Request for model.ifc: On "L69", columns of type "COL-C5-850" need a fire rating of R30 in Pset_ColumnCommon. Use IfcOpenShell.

First a look at what the model holds.

```python
import ifcopenshell
import ifcopenshell.util.element

model = ifcopenshell.open("model.ifc")
print(model.schema)
storey = next(s for s in model.by_type("IfcBuildingStorey") if s.Name == "L69")
columns = [e for e in ifcopenshell.util.element.get_decomposition(storey) if e.is_a("IfcColumn")]
seen = {}
for e in columns:
    element_type = ifcopenshell.util.element.get_type(e)
    key = (element_type.Name if element_type != e and element_type else None, ifcopenshell.util.element.get_pset(e, "Pset_ColumnCommon", "FireRating"))
    seen[key] = seen.get(key, 0) + 1
for (name, value), count in sorted(seen.items(), key=str):
    print(count, "x", name, "|", value)
```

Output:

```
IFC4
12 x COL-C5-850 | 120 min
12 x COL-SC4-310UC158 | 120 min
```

```python
import ifcopenshell
import ifcopenshell.api.pset
import ifcopenshell.util.element

model = ifcopenshell.open("model.ifc")

storey = next(s for s in model.by_type("IfcBuildingStorey") if s.Name == "L69")
columns = [e for e in ifcopenshell.util.element.get_decomposition(storey) if e.is_a("IfcColumn")]

count = 0
for e in columns:
    element_type = ifcopenshell.util.element.get_type(e)
    if element_type in (None, e) or element_type.Name != "COL-C5-850":
        continue
    # add_pset returns the element's existing set when there is one.
    pset = ifcopenshell.api.pset.add_pset(model, product=e, name="Pset_ColumnCommon")
    ifcopenshell.api.pset.edit_pset(model, pset=pset, properties={"FireRating": "R30"})
    count += 1

print(count, "columns updated")

model.write("model_v2.ifc")
```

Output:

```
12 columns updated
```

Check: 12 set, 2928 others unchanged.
